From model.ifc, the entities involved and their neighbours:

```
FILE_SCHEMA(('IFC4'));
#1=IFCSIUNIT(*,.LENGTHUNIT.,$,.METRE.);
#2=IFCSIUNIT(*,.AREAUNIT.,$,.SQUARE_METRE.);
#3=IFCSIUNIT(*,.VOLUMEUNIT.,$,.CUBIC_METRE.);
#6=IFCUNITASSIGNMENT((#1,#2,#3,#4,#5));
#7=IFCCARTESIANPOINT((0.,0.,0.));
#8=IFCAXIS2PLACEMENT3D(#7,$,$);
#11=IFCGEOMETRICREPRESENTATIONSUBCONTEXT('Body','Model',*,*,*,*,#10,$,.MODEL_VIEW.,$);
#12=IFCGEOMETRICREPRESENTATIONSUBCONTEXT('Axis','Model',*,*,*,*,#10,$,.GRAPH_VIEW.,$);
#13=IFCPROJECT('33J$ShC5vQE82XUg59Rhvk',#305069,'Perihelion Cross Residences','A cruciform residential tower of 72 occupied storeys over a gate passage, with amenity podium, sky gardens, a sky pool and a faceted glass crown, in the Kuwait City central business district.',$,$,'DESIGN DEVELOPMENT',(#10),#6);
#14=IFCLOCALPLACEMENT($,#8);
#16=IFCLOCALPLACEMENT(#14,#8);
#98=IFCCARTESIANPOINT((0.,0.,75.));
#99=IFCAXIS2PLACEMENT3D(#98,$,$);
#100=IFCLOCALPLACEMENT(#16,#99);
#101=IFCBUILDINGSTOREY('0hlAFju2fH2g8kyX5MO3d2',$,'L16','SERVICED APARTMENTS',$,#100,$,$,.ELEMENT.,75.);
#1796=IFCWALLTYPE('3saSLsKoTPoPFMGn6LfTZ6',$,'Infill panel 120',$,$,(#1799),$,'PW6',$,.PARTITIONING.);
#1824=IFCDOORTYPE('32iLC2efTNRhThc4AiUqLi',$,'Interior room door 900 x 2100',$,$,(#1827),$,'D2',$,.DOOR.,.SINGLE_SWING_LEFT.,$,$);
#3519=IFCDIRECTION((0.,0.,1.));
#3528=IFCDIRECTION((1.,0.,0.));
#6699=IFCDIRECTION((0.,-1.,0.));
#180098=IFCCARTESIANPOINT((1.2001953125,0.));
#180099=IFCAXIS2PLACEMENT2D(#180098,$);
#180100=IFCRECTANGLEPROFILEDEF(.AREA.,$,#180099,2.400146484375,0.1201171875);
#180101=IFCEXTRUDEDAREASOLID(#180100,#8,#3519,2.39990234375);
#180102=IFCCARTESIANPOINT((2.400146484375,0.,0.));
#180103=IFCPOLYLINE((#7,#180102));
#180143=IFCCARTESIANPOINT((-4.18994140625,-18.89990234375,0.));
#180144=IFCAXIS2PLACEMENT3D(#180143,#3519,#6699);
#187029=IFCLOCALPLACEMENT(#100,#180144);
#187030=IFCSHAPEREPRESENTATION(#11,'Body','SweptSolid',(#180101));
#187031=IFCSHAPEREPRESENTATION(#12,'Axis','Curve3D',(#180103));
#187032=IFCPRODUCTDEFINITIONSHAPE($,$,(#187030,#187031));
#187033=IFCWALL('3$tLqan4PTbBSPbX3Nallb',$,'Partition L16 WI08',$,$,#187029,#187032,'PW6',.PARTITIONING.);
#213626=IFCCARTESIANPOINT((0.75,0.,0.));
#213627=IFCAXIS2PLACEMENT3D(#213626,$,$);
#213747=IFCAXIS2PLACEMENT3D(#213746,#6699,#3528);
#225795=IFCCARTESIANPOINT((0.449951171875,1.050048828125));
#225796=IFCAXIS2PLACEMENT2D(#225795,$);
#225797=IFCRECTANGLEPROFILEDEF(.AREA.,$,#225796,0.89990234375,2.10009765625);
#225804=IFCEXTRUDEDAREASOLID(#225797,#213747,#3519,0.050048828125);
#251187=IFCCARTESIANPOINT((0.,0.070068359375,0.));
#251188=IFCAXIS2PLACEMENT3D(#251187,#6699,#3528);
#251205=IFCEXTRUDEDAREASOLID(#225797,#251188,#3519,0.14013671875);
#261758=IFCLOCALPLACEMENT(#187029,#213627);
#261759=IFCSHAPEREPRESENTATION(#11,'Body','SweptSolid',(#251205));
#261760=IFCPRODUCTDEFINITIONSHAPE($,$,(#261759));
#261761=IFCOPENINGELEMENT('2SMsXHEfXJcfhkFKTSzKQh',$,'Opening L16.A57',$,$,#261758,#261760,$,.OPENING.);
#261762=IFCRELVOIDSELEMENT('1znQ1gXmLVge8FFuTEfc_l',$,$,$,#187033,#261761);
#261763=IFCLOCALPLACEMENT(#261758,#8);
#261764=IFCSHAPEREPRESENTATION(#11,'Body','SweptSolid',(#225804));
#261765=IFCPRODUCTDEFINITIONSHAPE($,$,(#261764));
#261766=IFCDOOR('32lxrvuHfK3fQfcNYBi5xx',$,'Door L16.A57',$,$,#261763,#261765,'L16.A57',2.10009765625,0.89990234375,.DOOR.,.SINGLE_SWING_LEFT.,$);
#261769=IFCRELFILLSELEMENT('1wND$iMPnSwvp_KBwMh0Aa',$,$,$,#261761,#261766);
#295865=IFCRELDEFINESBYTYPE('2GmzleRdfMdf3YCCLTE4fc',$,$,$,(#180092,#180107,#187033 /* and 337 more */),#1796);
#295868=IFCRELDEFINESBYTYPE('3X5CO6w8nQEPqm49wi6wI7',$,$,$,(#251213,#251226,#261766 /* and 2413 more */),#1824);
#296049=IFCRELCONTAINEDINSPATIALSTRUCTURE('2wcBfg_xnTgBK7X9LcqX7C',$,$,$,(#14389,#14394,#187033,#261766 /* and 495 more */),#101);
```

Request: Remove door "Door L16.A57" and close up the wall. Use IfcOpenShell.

```python
import ifcopenshell
import ifcopenshell.api.feature
import ifcopenshell.api.root
import ifcopenshell.geom
import ifcopenshell.util.shape

model = ifcopenshell.open("model.ifc")
settings = ifcopenshell.geom.settings()


def volume(element):
    """Net volume in cubic metres, openings subtracted."""
    shape = ifcopenshell.geom.create_shape(settings, element)
    return ifcopenshell.util.shape.get_volume(shape.geometry)


door = model.by_id(261766)
opening = door.FillsVoids[0].RelatingOpeningElement
wall = opening.VoidsElements[0].RelatingBuildingElement
before = volume(wall)

ifcopenshell.api.root.remove_product(model, product=door)
ifcopenshell.api.feature.remove_feature(model, feature=opening)

after = volume(wall)

print(f"wall volume {before:.3f} -> {after:.3f} m3")

model.write("model_edited.ifc")
```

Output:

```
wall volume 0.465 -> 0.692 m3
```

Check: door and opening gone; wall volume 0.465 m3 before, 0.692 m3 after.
